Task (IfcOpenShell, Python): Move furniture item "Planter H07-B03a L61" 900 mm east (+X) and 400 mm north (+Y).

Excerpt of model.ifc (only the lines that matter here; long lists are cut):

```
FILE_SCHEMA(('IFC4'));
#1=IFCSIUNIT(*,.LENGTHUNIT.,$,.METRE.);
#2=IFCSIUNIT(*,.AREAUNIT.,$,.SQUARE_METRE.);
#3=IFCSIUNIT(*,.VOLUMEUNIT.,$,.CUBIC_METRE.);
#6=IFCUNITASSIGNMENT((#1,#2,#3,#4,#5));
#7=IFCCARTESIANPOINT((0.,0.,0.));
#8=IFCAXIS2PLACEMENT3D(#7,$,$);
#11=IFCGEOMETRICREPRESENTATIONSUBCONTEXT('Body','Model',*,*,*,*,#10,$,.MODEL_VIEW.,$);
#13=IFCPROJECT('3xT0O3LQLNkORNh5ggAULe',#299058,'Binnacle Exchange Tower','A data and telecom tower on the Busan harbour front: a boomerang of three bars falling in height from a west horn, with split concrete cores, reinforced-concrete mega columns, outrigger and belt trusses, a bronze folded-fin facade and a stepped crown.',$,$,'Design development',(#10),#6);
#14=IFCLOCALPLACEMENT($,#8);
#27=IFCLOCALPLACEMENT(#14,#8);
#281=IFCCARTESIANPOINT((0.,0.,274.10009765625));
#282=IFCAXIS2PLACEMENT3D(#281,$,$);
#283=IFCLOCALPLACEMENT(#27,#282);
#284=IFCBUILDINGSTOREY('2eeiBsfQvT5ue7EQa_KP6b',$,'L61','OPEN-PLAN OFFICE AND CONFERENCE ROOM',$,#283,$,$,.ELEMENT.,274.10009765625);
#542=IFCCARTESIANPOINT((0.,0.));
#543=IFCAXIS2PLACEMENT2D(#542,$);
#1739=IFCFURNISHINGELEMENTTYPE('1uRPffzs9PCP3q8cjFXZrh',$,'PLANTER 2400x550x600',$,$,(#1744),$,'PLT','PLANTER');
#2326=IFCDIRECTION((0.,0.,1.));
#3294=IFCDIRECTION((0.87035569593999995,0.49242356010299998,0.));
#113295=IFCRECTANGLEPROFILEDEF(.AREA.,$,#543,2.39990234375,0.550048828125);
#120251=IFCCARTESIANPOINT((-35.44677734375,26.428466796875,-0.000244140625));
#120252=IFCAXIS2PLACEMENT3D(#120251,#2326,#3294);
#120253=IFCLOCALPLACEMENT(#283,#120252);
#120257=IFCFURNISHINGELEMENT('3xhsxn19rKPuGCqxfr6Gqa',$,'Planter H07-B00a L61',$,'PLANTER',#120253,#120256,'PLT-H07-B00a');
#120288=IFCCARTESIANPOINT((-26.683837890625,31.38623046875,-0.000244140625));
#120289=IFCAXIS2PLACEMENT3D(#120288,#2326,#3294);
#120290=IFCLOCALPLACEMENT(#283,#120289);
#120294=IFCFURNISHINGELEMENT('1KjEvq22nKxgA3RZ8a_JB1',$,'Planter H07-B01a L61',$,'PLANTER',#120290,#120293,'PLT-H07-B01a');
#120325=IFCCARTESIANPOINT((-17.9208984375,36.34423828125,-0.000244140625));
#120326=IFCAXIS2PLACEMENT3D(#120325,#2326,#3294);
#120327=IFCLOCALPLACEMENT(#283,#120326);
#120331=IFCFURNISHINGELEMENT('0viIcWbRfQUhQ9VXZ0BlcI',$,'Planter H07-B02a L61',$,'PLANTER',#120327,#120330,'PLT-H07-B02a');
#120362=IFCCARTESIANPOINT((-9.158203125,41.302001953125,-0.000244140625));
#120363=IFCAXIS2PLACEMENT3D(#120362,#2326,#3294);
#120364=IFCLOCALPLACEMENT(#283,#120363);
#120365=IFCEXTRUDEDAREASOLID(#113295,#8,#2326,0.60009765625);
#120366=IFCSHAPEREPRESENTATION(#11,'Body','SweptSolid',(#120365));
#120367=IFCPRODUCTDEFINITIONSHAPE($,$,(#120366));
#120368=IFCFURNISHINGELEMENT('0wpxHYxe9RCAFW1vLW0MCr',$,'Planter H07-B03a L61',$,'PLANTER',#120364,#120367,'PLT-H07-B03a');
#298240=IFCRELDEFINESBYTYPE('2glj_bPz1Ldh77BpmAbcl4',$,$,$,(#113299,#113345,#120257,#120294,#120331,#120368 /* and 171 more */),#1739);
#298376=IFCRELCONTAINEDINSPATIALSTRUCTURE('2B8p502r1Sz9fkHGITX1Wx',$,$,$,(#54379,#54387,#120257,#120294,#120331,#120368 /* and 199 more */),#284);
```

```python
import ifcopenshell
import ifcopenshell.api.geometry
import ifcopenshell.util.placement
import ifcopenshell.util.unit

model = ifcopenshell.open("model.ifc")
unit_scale = ifcopenshell.util.unit.calculate_unit_scale(model)

item = model.by_id(120368)
matrix = ifcopenshell.util.placement.get_local_placement(item.ObjectPlacement)
matrix[0, 3] += 0.9 / unit_scale
matrix[1, 3] += 0.4 / unit_scale
ifcopenshell.api.geometry.edit_object_placement(model, product=item, matrix=matrix, is_si=False)

print(ifcopenshell.util.placement.get_local_placement(item.ObjectPlacement).round(3) + 0.0)

model.write("model-out.ifc")
```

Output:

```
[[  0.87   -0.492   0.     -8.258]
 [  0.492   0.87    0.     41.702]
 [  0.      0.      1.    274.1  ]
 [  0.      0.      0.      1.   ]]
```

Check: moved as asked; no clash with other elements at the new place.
